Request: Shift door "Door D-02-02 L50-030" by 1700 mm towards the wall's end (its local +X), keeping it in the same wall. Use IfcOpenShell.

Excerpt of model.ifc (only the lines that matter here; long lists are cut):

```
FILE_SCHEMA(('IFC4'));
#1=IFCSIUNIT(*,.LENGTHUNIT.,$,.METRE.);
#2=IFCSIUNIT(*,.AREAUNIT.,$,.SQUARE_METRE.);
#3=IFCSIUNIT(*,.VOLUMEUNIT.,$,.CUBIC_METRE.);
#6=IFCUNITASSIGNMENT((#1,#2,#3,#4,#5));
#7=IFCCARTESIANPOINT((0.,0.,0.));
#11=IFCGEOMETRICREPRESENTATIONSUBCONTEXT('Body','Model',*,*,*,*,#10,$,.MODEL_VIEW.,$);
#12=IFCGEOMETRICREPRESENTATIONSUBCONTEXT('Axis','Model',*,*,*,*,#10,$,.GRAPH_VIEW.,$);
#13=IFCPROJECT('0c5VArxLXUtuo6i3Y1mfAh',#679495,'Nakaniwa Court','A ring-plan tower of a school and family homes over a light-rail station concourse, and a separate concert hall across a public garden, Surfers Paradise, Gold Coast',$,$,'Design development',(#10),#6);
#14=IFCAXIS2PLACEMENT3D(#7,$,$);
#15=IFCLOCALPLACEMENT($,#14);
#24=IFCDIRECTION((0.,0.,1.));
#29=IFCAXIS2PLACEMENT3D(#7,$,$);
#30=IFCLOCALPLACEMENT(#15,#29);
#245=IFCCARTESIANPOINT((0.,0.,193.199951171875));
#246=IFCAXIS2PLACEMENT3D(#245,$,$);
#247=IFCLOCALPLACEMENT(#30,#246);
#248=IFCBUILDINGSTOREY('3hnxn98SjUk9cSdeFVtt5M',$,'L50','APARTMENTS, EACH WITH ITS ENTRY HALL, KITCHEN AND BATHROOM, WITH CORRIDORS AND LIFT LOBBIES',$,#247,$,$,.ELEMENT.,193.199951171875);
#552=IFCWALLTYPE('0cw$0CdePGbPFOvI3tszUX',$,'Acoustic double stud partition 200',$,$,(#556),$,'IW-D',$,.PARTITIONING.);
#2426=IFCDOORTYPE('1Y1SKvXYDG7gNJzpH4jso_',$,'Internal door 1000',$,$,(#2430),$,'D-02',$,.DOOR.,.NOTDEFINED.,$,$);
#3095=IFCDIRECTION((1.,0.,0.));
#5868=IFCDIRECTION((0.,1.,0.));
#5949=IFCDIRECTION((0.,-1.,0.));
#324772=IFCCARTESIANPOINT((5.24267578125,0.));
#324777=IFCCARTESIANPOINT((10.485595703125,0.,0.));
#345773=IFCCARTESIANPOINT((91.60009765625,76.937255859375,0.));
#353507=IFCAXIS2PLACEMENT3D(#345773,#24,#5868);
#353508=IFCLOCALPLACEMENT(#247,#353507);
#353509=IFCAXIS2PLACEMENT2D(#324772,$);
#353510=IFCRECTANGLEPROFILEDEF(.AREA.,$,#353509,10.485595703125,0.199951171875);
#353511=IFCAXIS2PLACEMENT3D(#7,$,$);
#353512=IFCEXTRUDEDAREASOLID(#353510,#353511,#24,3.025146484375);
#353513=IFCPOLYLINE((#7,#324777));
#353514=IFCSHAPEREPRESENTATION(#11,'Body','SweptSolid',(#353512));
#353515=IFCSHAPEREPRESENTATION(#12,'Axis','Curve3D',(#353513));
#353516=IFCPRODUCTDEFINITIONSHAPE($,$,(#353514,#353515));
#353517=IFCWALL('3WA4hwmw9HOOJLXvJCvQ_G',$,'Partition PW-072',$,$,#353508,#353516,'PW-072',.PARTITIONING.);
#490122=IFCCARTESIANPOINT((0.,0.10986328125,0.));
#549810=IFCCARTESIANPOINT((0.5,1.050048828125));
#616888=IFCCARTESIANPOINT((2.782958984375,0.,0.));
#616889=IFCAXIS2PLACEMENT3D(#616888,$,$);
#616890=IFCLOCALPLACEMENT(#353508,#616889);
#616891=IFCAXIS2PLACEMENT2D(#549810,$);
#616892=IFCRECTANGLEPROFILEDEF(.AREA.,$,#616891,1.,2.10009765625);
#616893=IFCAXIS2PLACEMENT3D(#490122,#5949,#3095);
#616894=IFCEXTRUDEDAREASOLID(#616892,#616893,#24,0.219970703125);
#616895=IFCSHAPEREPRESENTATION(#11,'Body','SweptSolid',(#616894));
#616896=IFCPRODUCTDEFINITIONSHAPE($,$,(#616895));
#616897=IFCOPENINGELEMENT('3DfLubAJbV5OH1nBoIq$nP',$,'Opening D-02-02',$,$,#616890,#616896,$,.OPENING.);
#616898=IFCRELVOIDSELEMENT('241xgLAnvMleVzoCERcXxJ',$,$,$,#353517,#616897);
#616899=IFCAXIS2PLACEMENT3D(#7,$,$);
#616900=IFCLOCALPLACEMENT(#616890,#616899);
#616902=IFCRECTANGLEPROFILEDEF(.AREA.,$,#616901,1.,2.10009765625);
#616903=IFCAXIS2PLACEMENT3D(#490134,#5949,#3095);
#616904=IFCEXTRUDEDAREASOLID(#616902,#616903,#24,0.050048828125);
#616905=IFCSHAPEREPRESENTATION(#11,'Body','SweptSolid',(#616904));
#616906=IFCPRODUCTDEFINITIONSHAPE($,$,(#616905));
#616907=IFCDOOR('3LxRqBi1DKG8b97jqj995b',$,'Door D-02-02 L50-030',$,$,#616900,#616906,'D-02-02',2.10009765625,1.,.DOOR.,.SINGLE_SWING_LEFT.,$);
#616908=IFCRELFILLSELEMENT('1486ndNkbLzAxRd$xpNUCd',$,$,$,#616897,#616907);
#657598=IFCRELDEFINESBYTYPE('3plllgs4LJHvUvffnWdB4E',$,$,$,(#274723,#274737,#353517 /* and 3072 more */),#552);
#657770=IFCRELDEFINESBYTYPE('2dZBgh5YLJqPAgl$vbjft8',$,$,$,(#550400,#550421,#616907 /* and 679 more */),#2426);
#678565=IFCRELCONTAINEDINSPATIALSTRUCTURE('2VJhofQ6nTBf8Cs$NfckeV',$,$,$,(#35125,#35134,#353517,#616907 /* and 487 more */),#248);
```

```python
import ifcopenshell
import ifcopenshell.api.geometry
import ifcopenshell.util.placement
import ifcopenshell.util.unit

model = ifcopenshell.open("model.ifc")
unit_scale = ifcopenshell.util.unit.calculate_unit_scale(model)

door = model.by_guid("3LxRqBi1DKG8b97jqj995b")
opening = door.FillsVoids[0].RelatingOpeningElement
wall = opening.VoidsElements[0].RelatingBuildingElement

wall_matrix = ifcopenshell.util.placement.get_local_placement(wall.ObjectPlacement)
shift = wall_matrix[:3, 0] * 1.7 / unit_scale
before = ifcopenshell.util.placement.get_local_placement(door.ObjectPlacement)[:3, 3].copy()

# The door is placed relative to its opening, so it follows when the opening moves.
matrix = ifcopenshell.util.placement.get_local_placement(opening.ObjectPlacement)
matrix[:3, 3] += shift
ifcopenshell.api.geometry.edit_object_placement(
    model, product=opening, matrix=matrix, is_si=False, should_transform_children=True
)

after = ifcopenshell.util.placement.get_local_placement(door.ObjectPlacement)[:3, 3]
print("door moved by", (after - before).round(3) + 0.0)

model.write("model_v2.ifc")
```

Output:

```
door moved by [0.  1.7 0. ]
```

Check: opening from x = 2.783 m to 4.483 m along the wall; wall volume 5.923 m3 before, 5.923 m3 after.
